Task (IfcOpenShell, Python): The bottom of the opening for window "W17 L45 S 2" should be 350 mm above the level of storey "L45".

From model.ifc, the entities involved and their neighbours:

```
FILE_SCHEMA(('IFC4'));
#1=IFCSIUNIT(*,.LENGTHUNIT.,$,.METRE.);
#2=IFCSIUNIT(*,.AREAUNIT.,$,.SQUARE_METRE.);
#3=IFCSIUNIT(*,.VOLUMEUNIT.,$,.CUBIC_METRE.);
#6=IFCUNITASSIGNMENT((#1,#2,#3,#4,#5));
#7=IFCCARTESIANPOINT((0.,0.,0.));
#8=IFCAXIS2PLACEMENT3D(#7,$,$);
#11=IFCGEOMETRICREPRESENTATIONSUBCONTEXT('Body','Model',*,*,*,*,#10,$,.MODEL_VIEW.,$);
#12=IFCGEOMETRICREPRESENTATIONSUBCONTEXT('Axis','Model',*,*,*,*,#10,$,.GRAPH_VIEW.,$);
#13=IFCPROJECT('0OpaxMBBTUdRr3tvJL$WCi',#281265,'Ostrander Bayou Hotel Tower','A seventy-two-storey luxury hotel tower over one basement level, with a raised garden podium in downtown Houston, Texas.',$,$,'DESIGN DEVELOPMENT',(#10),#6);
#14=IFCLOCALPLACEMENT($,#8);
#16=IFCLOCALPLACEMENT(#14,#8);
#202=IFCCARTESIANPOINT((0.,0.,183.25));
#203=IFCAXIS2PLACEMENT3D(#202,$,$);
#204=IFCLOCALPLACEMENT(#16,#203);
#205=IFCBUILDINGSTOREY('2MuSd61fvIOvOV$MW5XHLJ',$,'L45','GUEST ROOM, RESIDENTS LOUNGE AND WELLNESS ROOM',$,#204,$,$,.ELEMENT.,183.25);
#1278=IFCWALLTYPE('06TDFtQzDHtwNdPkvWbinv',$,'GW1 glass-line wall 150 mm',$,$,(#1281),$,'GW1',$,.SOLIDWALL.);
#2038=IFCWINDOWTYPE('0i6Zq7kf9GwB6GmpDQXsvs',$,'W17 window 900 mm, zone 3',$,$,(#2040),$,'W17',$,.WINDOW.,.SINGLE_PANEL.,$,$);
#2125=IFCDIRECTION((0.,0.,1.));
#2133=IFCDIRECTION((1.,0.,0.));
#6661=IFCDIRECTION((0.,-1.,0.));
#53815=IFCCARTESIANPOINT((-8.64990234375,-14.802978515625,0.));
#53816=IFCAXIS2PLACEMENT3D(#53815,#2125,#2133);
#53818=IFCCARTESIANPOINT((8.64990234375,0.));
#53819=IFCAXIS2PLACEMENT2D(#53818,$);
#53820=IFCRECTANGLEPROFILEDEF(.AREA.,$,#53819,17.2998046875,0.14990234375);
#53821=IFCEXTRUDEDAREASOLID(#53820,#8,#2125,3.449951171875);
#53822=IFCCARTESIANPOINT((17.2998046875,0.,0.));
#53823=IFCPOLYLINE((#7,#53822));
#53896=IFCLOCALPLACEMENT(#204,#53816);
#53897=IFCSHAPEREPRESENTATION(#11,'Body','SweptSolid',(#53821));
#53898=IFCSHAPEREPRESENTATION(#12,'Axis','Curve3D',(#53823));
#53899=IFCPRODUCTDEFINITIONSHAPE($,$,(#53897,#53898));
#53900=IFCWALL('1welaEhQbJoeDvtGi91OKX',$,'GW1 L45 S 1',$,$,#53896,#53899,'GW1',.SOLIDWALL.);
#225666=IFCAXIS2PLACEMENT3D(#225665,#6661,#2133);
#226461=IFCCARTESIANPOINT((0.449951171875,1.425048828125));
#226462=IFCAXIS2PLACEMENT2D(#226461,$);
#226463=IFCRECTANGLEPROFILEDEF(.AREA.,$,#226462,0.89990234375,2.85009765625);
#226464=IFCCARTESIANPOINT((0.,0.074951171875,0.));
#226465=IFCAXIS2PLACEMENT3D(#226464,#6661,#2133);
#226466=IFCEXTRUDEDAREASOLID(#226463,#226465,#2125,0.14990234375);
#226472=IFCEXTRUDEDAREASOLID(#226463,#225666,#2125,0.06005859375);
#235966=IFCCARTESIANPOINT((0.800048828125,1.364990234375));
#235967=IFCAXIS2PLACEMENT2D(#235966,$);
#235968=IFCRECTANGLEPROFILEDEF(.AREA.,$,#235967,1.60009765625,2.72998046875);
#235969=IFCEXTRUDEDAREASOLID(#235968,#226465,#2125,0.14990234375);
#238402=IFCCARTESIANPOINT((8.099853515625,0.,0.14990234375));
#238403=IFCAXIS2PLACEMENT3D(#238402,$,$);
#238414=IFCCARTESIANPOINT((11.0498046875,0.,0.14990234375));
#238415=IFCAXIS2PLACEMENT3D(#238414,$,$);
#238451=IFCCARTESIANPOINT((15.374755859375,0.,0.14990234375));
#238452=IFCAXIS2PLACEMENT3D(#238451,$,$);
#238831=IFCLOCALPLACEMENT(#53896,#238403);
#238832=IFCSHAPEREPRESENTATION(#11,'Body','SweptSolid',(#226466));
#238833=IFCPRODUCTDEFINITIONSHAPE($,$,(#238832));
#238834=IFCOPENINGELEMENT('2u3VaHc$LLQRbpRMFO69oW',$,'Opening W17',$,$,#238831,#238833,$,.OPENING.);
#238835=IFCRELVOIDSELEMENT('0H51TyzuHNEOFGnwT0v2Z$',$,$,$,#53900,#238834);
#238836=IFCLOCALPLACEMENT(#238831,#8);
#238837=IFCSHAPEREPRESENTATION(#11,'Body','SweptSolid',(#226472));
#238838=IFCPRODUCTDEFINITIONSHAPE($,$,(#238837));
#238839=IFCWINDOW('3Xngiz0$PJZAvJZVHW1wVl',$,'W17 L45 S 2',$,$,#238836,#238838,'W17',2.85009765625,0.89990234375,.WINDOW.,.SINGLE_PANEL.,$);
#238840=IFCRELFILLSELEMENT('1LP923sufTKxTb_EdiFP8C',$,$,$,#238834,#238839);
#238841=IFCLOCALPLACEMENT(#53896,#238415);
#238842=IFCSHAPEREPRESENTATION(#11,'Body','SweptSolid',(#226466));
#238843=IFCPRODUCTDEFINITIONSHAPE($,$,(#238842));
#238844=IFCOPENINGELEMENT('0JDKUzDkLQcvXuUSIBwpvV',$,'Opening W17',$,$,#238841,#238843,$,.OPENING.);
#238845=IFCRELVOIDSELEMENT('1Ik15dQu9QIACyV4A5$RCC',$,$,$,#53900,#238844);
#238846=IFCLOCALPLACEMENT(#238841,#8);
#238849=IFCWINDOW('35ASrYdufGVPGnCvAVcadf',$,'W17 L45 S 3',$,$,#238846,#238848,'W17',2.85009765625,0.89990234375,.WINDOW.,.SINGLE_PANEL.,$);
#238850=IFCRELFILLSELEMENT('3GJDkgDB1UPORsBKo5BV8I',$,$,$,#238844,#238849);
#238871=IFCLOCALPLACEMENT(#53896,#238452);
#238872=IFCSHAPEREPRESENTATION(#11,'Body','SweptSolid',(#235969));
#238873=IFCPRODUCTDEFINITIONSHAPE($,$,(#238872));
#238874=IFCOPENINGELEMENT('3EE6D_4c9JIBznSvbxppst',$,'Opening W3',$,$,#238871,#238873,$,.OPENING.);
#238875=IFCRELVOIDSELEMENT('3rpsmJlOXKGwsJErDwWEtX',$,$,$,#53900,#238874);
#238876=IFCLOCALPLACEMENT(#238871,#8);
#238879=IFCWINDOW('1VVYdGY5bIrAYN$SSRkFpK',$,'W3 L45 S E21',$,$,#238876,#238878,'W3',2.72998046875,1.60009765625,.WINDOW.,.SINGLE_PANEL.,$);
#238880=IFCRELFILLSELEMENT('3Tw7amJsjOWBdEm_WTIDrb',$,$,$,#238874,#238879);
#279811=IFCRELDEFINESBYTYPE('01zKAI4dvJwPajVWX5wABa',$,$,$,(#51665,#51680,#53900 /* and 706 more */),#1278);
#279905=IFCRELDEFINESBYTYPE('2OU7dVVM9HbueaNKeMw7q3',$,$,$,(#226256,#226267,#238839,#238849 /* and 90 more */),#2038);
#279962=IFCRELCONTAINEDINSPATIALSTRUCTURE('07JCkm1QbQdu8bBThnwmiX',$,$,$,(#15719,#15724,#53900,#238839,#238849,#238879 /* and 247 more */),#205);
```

```python
import numpy as np
import ifcopenshell
import ifcopenshell.api.geometry
import ifcopenshell.geom
import ifcopenshell.util.element
import ifcopenshell.util.placement
import ifcopenshell.util.shape
import ifcopenshell.util.unit

model = ifcopenshell.open("model.ifc")
unit_scale = ifcopenshell.util.unit.calculate_unit_scale(model)

window = model.by_guid("3Xngiz0$PJZAvJZVHW1wVl")
opening = window.FillsVoids[0].RelatingOpeningElement
storey = ifcopenshell.util.element.get_container(window, ifc_class="IfcBuildingStorey")
level = ifcopenshell.util.placement.get_local_placement(storey.ObjectPlacement)[2, 3]

# The opening's origin need not be at the sill, so measure its lowest point.
shape = ifcopenshell.geom.create_shape(ifcopenshell.geom.settings(), opening)
bottom = ifcopenshell.util.shape.get_shape_bottom_elevation(shape, shape.geometry) / unit_scale
dz = level + 0.35 / unit_scale - bottom

shift = np.array([0.0, 0.0, dz])
# The window is placed relative to its opening, so it follows when the opening moves.
matrix = ifcopenshell.util.placement.get_local_placement(opening.ObjectPlacement)
matrix[:3, 3] += shift
ifcopenshell.api.geometry.edit_object_placement(
    model, product=opening, matrix=matrix, is_si=False, should_transform_children=True
)

print(f"moved by {dz * unit_scale:+.3f} m")

model.write("model-out.ifc")
```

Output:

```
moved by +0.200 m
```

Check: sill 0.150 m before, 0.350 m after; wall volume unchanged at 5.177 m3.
